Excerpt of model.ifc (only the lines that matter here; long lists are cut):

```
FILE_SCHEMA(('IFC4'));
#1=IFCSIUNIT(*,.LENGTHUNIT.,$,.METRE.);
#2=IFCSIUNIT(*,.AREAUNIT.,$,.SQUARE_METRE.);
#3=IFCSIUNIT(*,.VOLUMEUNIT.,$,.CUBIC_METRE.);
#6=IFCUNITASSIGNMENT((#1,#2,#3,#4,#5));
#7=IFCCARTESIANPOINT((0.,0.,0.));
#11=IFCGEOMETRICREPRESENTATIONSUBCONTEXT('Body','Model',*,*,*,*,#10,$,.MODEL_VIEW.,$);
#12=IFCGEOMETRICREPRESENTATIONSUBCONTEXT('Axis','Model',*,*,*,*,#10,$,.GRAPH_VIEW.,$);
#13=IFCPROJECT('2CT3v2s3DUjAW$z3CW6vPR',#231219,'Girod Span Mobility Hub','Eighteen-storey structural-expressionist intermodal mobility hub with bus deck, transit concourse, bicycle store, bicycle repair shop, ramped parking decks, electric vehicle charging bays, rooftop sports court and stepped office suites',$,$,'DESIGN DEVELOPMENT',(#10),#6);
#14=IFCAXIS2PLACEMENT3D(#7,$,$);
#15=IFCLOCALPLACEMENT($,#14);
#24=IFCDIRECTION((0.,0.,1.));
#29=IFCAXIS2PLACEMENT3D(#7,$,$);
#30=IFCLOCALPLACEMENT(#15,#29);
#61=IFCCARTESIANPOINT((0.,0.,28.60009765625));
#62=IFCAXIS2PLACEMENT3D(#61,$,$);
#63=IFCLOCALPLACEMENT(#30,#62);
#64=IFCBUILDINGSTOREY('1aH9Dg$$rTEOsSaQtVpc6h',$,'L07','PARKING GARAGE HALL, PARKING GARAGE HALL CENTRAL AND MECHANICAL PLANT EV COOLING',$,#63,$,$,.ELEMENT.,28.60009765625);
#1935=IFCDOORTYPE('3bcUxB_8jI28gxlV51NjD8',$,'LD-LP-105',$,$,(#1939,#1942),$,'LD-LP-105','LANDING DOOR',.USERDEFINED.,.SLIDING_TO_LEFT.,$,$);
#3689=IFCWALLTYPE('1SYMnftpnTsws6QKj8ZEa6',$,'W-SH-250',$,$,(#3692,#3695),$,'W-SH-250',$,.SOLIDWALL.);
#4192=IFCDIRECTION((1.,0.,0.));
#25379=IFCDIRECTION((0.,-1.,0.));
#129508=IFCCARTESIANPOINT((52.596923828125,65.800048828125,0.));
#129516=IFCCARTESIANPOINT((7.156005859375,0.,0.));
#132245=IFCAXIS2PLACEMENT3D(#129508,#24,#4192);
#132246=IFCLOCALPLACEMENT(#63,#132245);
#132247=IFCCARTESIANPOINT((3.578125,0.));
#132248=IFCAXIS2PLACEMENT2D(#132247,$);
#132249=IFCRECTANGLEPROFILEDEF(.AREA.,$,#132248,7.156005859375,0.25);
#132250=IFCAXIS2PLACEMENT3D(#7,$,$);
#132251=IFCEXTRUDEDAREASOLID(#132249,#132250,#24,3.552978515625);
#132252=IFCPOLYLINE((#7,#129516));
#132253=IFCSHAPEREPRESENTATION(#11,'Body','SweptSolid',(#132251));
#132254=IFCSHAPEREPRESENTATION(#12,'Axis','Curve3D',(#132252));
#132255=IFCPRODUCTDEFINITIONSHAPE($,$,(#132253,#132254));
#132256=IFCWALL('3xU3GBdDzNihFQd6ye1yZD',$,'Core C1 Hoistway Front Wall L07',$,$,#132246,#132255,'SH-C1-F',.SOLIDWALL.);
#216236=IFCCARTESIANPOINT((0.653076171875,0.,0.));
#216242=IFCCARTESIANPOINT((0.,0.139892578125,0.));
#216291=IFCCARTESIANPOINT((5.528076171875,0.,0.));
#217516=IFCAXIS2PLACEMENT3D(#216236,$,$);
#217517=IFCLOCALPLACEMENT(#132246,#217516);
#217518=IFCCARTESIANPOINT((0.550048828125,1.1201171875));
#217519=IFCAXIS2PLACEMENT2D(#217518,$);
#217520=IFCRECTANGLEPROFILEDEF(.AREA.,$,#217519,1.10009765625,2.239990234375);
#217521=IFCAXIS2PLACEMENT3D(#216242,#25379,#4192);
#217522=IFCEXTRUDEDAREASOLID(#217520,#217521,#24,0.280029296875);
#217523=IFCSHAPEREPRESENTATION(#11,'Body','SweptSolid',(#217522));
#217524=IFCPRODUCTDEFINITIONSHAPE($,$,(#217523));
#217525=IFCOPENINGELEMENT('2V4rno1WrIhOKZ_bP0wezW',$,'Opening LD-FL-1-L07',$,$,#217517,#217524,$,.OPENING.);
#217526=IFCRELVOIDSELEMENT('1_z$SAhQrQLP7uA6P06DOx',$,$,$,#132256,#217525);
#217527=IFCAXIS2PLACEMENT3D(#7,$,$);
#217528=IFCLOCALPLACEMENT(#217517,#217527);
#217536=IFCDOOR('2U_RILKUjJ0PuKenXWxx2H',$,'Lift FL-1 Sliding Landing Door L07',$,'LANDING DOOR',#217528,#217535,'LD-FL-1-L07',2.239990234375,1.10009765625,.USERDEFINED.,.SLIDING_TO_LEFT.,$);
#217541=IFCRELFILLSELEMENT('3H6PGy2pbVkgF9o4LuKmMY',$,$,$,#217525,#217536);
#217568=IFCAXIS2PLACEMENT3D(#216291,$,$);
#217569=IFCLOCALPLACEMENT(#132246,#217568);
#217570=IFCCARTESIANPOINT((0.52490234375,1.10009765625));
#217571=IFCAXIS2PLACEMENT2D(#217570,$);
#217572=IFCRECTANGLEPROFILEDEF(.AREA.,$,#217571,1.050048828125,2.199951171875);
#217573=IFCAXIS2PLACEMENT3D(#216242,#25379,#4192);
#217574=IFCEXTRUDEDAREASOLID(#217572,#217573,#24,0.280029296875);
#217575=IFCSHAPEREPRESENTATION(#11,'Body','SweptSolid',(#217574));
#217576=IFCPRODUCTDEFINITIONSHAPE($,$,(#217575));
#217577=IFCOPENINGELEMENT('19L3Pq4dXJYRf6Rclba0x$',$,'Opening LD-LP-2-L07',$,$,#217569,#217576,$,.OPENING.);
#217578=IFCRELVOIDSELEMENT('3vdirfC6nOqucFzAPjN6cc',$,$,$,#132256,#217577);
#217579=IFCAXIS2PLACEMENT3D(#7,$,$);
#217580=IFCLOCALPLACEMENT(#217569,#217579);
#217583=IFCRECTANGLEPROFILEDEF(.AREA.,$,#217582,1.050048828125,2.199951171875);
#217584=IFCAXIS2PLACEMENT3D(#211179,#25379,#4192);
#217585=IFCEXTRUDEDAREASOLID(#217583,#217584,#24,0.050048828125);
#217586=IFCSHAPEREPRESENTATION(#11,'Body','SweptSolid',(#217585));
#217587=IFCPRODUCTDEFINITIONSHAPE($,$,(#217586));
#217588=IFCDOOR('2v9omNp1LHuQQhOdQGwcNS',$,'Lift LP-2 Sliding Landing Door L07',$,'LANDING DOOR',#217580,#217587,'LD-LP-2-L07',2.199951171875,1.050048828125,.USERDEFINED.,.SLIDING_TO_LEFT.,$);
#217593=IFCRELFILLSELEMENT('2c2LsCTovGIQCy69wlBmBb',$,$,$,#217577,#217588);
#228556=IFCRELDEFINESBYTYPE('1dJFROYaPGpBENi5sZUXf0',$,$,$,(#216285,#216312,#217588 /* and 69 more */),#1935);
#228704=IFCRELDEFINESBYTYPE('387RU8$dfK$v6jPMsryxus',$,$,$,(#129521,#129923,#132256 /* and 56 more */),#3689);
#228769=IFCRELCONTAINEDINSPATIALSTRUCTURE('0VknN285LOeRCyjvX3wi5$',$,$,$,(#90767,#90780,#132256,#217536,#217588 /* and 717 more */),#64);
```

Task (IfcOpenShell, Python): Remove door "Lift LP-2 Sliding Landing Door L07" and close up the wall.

```python
import ifcopenshell
import ifcopenshell.api.feature
import ifcopenshell.api.root
import ifcopenshell.geom
import ifcopenshell.util.shape

model = ifcopenshell.open("model.ifc")
settings = ifcopenshell.geom.settings()


def volume(element):
    """Net volume in cubic metres, openings subtracted."""
    shape = ifcopenshell.geom.create_shape(settings, element)
    return ifcopenshell.util.shape.get_volume(shape.geometry)


door = model.by_id(217588)
opening = door.FillsVoids[0].RelatingOpeningElement
wall = opening.VoidsElements[0].RelatingBuildingElement
before = volume(wall)

ifcopenshell.api.root.remove_product(model, product=door)
ifcopenshell.api.feature.remove_feature(model, feature=opening)

after = volume(wall)

print(f"wall volume {before:.3f} -> {after:.3f} m3")

model.write("model_updated.ifc")
```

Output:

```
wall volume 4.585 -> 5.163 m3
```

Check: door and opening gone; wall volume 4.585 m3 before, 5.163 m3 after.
